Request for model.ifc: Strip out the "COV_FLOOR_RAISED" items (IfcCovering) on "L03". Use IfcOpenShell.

First a look at what the model holds.

```python
import ifcopenshell
import ifcopenshell.util.element

model = ifcopenshell.open("model.ifc")
print(model.schema)
storey = next(s for s in model.by_type("IfcBuildingStorey") if s.Name == "L03")
coverings = [e for e in ifcopenshell.util.element.get_decomposition(storey) if e.is_a("IfcCovering")]
seen = {}
for e in coverings:
    element_type = ifcopenshell.util.element.get_type(e)
    name = element_type.Name if element_type not in (None, e) else None
    seen[name] = seen.get(name, 0) + 1
for name, count in sorted(seen.items(), key=str):
    print(count, "x", name)
```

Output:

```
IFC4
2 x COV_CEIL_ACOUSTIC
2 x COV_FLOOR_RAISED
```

```python
import ifcopenshell
import ifcopenshell.api.root
import ifcopenshell.util.element

model = ifcopenshell.open("model.ifc")

storey = next(s for s in model.by_type("IfcBuildingStorey") if s.Name == "L03")
coverings = [e for e in ifcopenshell.util.element.get_decomposition(storey) if e.is_a("IfcCovering")]
targets = [e for e in coverings if (t := ifcopenshell.util.element.get_type(e)) not in (None, e) and t.Name == "COV_FLOOR_RAISED"]

for e in targets:
    ifcopenshell.api.root.remove_product(model, product=e)
print(len(targets), "removed")

model.write("model_updated.ifc")
```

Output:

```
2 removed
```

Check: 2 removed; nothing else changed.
